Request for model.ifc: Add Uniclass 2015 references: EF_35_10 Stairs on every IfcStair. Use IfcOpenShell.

First a look at what the model holds.

```python
import ifcopenshell

model = ifcopenshell.open("model.ifc")
print(model.schema)
print("classifications:", [c.Name for c in model.by_type("IfcClassification")])
for ifc_class in ("IfcDoor", "IfcRoof", "IfcStair", "IfcWall", "IfcWindow"):
    print(ifc_class, len(model.by_type(ifc_class)))
```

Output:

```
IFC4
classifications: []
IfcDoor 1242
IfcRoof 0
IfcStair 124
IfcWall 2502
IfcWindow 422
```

```python
import ifcopenshell
import ifcopenshell.api.classification

model = ifcopenshell.open("model.ifc")

system = ifcopenshell.api.classification.add_classification(model, classification="Uniclass 2015")

codes = {
    "IfcStair": ("EF_35_10", "Stairs"),
}
for ifc_class, (code, name) in codes.items():
    products = model.by_type(ifc_class)
    ifcopenshell.api.classification.add_reference(
        model, products=products, classification=system, identification=code, name=name
    )
    print(code, len(products))

model.write("model_updated.ifc")
```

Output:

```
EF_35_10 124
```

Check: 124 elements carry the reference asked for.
